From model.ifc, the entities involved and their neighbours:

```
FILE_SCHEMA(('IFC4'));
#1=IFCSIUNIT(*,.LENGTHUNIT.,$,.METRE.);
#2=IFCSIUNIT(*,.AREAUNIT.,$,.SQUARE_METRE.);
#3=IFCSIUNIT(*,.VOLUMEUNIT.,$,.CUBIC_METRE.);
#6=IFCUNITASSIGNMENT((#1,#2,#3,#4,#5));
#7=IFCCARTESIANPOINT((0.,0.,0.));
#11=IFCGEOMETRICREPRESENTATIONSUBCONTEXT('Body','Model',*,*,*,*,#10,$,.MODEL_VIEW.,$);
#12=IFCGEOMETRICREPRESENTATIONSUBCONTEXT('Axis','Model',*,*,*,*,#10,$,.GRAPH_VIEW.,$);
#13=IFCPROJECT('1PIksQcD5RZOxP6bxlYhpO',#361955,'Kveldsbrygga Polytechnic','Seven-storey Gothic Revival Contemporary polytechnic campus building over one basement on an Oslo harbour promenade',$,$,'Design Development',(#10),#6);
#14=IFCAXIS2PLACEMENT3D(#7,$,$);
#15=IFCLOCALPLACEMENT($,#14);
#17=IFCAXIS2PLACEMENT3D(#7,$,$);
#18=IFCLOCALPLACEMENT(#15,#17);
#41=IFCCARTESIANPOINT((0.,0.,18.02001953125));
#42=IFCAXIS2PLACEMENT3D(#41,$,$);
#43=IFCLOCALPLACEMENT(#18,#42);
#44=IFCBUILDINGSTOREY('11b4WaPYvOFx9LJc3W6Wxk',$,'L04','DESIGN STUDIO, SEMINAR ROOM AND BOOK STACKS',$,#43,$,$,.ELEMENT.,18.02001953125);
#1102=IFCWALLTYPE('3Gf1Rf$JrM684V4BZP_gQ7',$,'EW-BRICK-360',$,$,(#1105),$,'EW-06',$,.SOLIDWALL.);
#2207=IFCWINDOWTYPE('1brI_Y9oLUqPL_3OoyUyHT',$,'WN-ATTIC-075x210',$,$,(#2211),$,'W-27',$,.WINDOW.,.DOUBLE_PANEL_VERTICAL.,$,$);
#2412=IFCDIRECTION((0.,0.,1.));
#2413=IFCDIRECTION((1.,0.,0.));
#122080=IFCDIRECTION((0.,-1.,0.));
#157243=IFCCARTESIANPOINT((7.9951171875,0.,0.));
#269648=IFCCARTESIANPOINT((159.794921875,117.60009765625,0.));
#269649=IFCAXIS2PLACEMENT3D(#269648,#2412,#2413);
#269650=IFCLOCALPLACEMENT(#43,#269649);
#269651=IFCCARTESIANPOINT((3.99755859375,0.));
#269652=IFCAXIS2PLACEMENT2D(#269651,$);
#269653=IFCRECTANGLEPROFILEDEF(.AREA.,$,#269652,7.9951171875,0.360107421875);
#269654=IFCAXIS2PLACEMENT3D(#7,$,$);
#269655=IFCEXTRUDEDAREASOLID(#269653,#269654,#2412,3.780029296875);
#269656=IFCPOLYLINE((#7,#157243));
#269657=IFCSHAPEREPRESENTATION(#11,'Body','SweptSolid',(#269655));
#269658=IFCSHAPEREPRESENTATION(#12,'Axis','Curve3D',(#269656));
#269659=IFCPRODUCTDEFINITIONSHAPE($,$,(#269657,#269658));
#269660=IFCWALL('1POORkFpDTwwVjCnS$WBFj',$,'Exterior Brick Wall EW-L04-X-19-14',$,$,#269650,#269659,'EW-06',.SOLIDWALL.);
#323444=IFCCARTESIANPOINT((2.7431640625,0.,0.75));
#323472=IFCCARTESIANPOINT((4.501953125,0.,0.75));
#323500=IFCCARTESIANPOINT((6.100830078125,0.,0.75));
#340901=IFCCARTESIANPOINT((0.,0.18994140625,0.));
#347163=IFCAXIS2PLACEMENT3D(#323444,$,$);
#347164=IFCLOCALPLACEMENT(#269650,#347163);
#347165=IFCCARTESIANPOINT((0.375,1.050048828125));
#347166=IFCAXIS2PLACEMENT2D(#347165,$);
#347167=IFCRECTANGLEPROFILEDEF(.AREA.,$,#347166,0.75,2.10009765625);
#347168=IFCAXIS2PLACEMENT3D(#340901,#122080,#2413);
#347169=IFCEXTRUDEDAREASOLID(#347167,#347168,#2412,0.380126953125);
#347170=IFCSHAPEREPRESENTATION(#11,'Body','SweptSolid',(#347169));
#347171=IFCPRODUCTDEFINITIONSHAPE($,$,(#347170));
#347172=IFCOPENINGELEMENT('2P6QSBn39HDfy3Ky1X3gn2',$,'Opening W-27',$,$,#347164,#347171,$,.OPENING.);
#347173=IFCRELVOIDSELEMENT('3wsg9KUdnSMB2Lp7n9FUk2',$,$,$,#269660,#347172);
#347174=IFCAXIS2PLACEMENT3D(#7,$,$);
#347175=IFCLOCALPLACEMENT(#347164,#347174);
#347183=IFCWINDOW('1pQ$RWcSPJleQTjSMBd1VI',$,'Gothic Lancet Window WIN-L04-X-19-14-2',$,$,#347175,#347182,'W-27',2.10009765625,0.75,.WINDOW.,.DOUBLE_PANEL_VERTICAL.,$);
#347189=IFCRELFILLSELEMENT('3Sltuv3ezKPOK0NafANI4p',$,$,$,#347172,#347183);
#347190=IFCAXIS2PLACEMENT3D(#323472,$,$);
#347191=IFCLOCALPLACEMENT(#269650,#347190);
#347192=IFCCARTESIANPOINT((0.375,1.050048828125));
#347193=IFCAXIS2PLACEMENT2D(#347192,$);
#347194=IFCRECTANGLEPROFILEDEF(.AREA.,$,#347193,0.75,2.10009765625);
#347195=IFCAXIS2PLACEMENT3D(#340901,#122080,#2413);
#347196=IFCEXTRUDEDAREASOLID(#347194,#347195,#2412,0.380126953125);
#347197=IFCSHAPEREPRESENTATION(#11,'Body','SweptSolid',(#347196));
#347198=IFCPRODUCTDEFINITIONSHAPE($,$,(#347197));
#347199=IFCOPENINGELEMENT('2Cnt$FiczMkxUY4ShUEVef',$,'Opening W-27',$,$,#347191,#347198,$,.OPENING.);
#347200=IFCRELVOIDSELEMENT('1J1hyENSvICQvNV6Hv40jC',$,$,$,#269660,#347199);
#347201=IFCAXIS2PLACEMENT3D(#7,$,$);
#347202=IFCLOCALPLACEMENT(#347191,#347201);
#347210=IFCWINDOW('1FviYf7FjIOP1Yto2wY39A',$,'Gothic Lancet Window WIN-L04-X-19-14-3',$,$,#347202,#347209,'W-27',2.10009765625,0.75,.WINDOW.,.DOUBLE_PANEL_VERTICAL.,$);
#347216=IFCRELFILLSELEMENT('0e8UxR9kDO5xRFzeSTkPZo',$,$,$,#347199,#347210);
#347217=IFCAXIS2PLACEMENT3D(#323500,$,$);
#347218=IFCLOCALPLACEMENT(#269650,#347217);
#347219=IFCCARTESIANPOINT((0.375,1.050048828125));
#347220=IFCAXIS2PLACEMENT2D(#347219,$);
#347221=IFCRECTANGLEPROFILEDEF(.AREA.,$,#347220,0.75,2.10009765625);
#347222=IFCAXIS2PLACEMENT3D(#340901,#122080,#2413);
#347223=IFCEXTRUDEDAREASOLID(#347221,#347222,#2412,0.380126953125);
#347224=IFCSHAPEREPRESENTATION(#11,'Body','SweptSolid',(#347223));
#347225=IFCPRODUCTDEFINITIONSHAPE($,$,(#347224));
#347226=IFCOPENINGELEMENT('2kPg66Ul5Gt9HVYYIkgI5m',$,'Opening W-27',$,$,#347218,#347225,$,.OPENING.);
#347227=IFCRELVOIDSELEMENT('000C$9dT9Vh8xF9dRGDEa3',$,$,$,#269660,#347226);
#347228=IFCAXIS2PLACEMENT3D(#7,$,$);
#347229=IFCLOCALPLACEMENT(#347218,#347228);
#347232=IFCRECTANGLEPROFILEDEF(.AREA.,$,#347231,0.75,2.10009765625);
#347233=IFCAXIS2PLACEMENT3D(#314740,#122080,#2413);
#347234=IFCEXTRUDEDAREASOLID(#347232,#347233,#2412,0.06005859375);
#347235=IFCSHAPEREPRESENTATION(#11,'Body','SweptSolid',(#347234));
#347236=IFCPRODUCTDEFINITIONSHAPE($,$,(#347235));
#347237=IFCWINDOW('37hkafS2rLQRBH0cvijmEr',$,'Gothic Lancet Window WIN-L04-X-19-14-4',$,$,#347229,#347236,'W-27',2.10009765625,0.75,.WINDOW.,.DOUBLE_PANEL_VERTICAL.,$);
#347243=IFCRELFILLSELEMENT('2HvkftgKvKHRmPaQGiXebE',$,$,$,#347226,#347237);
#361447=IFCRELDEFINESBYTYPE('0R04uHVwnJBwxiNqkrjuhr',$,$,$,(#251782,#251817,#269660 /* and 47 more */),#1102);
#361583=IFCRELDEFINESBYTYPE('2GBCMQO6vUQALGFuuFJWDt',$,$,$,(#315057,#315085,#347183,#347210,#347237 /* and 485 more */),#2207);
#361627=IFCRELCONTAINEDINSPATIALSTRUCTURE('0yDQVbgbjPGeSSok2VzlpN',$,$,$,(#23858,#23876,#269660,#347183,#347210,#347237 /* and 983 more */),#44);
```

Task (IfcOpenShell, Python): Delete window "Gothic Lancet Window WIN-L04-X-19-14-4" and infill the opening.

```python
import ifcopenshell
import ifcopenshell.api.feature
import ifcopenshell.api.root
import ifcopenshell.geom
import ifcopenshell.util.shape

model = ifcopenshell.open("model.ifc")
settings = ifcopenshell.geom.settings()


def volume(element):
    """Net volume in cubic metres, openings subtracted."""
    shape = ifcopenshell.geom.create_shape(settings, element)
    return ifcopenshell.util.shape.get_volume(shape.geometry)


window = model.by_id(347237)
opening = window.FillsVoids[0].RelatingOpeningElement
wall = opening.VoidsElements[0].RelatingBuildingElement
before = volume(wall)

ifcopenshell.api.root.remove_product(model, product=window)
ifcopenshell.api.feature.remove_feature(model, feature=opening)

after = volume(wall)

print(f"wall volume {before:.3f} -> {after:.3f} m3")

model.write("model_v2.ifc")
```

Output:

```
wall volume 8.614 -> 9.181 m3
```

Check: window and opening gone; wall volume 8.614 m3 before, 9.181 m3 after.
